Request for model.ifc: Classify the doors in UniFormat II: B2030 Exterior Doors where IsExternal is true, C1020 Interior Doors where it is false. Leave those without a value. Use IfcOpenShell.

First a look at what the model holds.

```python
import ifcopenshell
import ifcopenshell.util.element

model = ifcopenshell.open("model.ifc")
print(model.schema)
print("classifications:", [c.Name for c in model.by_type("IfcClassification")])
values = [ifcopenshell.util.element.get_pset(e, "Pset_DoorCommon", "IsExternal") for e in model.by_type("IfcDoor")]
for value in (True, False, None):
    print("IsExternal", value, values.count(value))
```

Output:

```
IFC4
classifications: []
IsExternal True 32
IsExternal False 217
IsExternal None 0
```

```python
import ifcopenshell
import ifcopenshell.api.classification
import ifcopenshell.util.element

model = ifcopenshell.open("model.ifc")

system = ifcopenshell.api.classification.add_classification(model, classification="UniFormat II")

doors = model.by_type("IfcDoor")
external = {e: ifcopenshell.util.element.get_pset(e, "Pset_DoorCommon", "IsExternal") for e in doors}
for flag, code, name in ((True, "B2030", "Exterior Doors"), (False, "C1020", "Interior Doors")):
    products = [e for e in doors if external[e] is flag]
    ifcopenshell.api.classification.add_reference(
        model, products=products, classification=system, identification=code, name=name
    )
    print(code, len(products))

model.write("model_edited.ifc")
```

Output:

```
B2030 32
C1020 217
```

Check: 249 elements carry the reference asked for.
